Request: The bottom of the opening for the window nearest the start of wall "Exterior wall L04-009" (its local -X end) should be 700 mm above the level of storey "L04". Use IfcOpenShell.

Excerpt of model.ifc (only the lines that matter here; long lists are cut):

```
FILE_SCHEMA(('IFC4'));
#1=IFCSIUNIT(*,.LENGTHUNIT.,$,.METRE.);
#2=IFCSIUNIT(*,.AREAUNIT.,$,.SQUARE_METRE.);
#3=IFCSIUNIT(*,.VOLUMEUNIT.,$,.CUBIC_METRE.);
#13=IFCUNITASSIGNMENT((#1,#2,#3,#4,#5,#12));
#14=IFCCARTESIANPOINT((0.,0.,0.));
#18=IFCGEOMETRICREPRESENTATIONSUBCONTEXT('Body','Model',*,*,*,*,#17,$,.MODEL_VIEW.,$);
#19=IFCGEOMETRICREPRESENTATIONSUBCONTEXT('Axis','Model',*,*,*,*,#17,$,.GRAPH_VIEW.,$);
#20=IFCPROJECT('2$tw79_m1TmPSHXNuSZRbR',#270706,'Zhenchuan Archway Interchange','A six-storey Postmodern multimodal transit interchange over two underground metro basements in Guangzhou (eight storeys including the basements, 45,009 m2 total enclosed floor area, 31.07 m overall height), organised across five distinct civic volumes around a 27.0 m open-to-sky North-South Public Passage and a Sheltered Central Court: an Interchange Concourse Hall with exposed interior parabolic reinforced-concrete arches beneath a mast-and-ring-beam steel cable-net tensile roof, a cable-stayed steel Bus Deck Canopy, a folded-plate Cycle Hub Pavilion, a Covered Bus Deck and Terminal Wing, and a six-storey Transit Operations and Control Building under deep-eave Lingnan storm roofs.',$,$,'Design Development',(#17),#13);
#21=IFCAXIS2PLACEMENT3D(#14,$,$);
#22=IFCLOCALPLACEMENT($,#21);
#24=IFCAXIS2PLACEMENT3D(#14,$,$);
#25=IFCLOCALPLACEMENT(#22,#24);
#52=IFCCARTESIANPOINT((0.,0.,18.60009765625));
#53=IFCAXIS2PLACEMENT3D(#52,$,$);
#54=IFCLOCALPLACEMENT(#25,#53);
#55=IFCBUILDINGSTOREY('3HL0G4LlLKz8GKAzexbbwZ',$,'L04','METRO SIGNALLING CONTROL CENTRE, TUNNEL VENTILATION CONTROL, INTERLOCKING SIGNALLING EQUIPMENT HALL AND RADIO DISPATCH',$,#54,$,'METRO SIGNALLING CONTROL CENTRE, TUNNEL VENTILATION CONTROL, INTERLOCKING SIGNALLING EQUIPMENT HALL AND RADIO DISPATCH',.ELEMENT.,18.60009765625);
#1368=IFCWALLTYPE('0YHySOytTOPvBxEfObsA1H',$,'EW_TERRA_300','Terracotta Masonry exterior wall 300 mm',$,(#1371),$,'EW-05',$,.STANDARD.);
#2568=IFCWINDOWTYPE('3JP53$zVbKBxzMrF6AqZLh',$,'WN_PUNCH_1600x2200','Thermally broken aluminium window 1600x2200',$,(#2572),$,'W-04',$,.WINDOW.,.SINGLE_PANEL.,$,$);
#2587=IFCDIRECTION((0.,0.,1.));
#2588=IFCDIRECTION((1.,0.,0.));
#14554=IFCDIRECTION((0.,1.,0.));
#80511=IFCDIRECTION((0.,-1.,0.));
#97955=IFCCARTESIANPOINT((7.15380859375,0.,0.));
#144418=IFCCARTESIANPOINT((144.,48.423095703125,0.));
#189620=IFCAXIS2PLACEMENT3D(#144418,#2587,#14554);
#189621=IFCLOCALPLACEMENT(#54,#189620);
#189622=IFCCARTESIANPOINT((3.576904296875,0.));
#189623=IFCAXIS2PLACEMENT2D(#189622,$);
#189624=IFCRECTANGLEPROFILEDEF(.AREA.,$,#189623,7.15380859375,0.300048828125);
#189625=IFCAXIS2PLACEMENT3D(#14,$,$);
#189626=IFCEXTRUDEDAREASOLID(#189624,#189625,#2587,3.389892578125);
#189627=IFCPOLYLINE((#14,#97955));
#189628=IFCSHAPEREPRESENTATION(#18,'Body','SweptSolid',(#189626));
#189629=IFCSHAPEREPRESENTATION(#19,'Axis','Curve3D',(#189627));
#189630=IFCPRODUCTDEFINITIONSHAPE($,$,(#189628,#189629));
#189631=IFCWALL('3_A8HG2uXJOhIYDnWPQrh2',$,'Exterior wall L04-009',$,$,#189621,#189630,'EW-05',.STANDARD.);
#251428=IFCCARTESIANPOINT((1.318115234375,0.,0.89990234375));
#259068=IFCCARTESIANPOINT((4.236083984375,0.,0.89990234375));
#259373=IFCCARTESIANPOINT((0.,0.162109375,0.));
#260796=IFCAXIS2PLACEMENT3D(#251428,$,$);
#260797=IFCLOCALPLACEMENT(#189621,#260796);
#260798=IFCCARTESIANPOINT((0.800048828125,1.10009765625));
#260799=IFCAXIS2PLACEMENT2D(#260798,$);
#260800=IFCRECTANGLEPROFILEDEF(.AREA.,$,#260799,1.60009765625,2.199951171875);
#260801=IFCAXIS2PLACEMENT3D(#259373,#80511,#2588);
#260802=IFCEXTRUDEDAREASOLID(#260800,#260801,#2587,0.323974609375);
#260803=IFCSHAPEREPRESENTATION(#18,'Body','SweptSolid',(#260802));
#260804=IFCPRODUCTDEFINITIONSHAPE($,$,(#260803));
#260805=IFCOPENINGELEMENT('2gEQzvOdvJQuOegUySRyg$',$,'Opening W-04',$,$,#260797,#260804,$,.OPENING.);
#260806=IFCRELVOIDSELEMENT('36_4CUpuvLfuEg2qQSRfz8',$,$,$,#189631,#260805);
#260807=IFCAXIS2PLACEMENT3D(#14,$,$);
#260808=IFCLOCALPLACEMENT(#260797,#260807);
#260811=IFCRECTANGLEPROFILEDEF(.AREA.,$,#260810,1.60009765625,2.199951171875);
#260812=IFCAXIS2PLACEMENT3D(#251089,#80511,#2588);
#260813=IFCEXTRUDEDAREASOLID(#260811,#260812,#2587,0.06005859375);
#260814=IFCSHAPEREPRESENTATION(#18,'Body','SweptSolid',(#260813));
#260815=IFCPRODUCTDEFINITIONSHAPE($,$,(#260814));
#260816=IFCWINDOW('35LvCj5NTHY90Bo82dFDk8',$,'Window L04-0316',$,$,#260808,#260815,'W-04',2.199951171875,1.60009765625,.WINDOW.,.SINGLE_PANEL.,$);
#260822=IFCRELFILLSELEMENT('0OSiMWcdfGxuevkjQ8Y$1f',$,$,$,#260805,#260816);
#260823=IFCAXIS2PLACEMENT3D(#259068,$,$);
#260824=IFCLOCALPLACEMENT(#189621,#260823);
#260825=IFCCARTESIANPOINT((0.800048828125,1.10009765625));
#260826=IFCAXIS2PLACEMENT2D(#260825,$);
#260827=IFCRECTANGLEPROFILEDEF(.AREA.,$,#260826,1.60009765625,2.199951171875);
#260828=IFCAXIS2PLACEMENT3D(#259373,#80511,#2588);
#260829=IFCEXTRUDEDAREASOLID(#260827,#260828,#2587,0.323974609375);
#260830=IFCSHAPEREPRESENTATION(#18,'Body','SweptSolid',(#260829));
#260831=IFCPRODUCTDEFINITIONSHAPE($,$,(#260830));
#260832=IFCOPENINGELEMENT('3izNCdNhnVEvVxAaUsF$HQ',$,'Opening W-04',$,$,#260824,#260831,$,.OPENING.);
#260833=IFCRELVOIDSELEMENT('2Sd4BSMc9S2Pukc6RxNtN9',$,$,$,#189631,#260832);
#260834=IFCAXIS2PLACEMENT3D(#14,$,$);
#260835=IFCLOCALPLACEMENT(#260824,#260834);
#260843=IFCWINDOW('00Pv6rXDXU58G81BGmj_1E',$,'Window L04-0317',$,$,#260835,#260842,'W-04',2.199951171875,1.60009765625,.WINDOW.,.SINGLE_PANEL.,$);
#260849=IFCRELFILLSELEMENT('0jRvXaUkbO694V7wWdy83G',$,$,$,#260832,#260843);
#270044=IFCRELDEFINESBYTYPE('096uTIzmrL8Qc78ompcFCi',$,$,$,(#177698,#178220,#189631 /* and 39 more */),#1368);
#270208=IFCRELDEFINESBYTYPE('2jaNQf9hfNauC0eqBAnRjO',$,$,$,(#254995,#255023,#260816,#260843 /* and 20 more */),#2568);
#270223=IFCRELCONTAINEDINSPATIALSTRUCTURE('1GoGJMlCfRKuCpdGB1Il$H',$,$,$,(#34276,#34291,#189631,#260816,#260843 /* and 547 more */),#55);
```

```python
import numpy as np
import ifcopenshell
import ifcopenshell.api.geometry
import ifcopenshell.geom
import ifcopenshell.util.element
import ifcopenshell.util.placement
import ifcopenshell.util.shape
import ifcopenshell.util.unit

model = ifcopenshell.open("model.ifc")
unit_scale = ifcopenshell.util.unit.calculate_unit_scale(model)

window = model.by_guid("35LvCj5NTHY90Bo82dFDk8")
opening = window.FillsVoids[0].RelatingOpeningElement
storey = ifcopenshell.util.element.get_container(window, ifc_class="IfcBuildingStorey")
level = ifcopenshell.util.placement.get_local_placement(storey.ObjectPlacement)[2, 3]

# The opening's origin need not be at the sill, so measure its lowest point.
shape = ifcopenshell.geom.create_shape(ifcopenshell.geom.settings(), opening)
bottom = ifcopenshell.util.shape.get_shape_bottom_elevation(shape, shape.geometry) / unit_scale
dz = level + 0.7 / unit_scale - bottom

shift = np.array([0.0, 0.0, dz])
# The window is placed relative to its opening, so it follows when the opening moves.
matrix = ifcopenshell.util.placement.get_local_placement(opening.ObjectPlacement)
matrix[:3, 3] += shift
ifcopenshell.api.geometry.edit_object_placement(
    model, product=opening, matrix=matrix, is_si=False, should_transform_children=True
)

print(f"moved by {dz * unit_scale:+.3f} m")

model.write("model-out.ifc")
```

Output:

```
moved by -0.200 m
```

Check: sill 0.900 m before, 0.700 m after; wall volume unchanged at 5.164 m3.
